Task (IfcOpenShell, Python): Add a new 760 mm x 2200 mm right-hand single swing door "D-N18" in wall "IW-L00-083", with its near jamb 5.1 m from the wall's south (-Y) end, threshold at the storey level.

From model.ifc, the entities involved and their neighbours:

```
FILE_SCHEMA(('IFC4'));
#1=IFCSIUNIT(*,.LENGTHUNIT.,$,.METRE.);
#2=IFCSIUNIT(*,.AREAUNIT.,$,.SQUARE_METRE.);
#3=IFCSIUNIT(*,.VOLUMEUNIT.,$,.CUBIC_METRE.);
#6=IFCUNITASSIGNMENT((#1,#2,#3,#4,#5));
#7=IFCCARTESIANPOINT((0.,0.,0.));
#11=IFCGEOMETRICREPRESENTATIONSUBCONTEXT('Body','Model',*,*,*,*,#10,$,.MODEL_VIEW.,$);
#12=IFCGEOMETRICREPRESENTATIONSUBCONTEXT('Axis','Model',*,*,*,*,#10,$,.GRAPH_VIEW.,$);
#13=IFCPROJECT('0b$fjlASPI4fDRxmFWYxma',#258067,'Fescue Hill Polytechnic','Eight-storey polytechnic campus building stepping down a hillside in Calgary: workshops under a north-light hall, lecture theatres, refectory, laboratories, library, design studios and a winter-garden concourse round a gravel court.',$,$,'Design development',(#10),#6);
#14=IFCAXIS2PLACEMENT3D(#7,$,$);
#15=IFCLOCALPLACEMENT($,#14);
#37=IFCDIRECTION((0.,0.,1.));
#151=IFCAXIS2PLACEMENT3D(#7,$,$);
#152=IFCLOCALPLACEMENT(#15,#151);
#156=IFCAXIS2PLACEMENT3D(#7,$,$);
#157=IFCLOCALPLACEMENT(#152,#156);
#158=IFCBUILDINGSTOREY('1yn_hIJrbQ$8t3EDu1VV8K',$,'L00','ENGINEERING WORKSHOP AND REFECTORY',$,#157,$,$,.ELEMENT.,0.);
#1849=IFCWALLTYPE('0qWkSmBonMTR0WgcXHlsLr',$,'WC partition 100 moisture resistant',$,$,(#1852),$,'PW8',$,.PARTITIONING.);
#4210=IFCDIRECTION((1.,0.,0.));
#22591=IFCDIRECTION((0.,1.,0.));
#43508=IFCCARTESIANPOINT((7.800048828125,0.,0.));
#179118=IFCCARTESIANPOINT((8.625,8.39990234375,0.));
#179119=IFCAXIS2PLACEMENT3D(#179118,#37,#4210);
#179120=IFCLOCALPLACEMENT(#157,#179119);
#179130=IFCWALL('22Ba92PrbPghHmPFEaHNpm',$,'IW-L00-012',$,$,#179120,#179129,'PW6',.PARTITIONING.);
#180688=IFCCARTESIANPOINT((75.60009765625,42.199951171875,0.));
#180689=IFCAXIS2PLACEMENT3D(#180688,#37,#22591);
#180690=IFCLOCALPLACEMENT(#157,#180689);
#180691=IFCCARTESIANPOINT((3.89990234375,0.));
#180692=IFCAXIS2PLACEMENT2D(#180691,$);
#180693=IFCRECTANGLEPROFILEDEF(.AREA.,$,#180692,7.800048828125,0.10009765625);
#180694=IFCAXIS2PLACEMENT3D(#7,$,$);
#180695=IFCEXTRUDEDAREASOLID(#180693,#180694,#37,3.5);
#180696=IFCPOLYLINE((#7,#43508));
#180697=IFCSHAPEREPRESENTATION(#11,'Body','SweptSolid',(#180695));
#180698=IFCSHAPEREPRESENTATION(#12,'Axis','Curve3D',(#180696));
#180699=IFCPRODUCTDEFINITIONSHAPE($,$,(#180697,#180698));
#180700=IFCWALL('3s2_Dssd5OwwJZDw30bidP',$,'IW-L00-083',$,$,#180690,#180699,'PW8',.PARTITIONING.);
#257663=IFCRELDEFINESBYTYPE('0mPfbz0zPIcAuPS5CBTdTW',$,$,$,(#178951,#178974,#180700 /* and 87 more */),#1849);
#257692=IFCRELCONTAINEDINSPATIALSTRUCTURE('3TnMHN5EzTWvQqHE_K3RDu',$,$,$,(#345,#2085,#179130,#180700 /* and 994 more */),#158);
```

```python
import numpy as np
import ifcopenshell
import ifcopenshell.api.feature
import ifcopenshell.api.geometry
import ifcopenshell.api.root
import ifcopenshell.api.spatial
import ifcopenshell.geom
import ifcopenshell.util.element
import ifcopenshell.util.placement
import ifcopenshell.util.representation
import ifcopenshell.util.shape
import ifcopenshell.util.unit

model = ifcopenshell.open("model.ifc")
unit_scale = ifcopenshell.util.unit.calculate_unit_scale(model)
settings = ifcopenshell.geom.settings()


def volume(element):
    """Net volume in cubic metres, openings subtracted."""
    shape = ifcopenshell.geom.create_shape(settings, element)
    return ifcopenshell.util.shape.get_volume(shape.geometry)


wall = model.by_guid("3s2_Dssd5OwwJZDw30bidP")
storey = ifcopenshell.util.element.get_container(wall, ifc_class="IfcBuildingStorey")
context = ifcopenshell.util.representation.get_context(model, "Model", "Body", "MODEL_VIEW")
before = volume(wall)

width, height, from_end, sill = 0.76, 2.2, 5.1, 0.0  # metres

# The wall runs along its own X axis, and the end named is its -X end.
wall_shape = ifcopenshell.geom.create_shape(settings, wall)
x, y, z = ifcopenshell.util.shape.get_vertices(wall_shape.geometry).T
start = x.min() + from_end
face, thickness = float(y.min()), float(y.max() - y.min())
wall_matrix = ifcopenshell.util.placement.get_local_placement(wall.ObjectPlacement)
level = ifcopenshell.util.placement.get_local_placement(storey.ObjectPlacement)[2, 3]


def in_wall(x, y):
    """Placement at x, y metres in the wall's axes, at sill height."""
    matrix = wall_matrix.copy()
    matrix[:, 3] = wall_matrix @ np.array([x / unit_scale, y / unit_scale, 0.0, 1.0])
    matrix[2, 3] = level + sill / unit_scale
    return matrix


# Opening: a box that overshoots both wall faces by 50 mm.
opening = ifcopenshell.api.root.create_entity(model, ifc_class="IfcOpeningElement", predefined_type="OPENING")
box = ifcopenshell.api.geometry.add_wall_representation(
    model, context=context, length=width, height=height, thickness=thickness + 0.1
)
ifcopenshell.api.geometry.assign_representation(model, product=opening, representation=box)
ifcopenshell.api.geometry.edit_object_placement(model, product=opening, matrix=in_wall(start, face - 0.05), is_si=False)
ifcopenshell.api.feature.add_feature(model, feature=opening, element=wall)

door = ifcopenshell.api.root.create_entity(model, ifc_class="IfcDoor", name="D-N18", predefined_type="DOOR")
door.OverallWidth, door.OverallHeight = width / unit_scale, height / unit_scale
door.OperationType = "SINGLE_SWING_RIGHT"
body = ifcopenshell.api.geometry.add_door_representation(
    model,
    context=context,
    overall_width=door.OverallWidth,
    overall_height=door.OverallHeight,
    operation_type="SINGLE_SWING_RIGHT",
    lining_properties={"LiningDepth": thickness / unit_scale, "ThresholdDepth": thickness / unit_scale},
)
ifcopenshell.api.geometry.assign_representation(model, product=door, representation=body)
ifcopenshell.api.spatial.assign_container(model, products=[door], relating_structure=storey)
ifcopenshell.api.feature.add_filling(model, opening=opening, element=door)

# The lining spans the wall, so the door starts at the wall face.
ifcopenshell.api.geometry.edit_object_placement(model, product=door, matrix=in_wall(start, face), is_si=False)

after = volume(wall)

print(f"wall volume {before:.3f} -> {after:.3f} m3")

model.write("model_updated.ifc")
```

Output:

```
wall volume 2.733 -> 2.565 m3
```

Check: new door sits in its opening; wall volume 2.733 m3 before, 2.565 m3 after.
